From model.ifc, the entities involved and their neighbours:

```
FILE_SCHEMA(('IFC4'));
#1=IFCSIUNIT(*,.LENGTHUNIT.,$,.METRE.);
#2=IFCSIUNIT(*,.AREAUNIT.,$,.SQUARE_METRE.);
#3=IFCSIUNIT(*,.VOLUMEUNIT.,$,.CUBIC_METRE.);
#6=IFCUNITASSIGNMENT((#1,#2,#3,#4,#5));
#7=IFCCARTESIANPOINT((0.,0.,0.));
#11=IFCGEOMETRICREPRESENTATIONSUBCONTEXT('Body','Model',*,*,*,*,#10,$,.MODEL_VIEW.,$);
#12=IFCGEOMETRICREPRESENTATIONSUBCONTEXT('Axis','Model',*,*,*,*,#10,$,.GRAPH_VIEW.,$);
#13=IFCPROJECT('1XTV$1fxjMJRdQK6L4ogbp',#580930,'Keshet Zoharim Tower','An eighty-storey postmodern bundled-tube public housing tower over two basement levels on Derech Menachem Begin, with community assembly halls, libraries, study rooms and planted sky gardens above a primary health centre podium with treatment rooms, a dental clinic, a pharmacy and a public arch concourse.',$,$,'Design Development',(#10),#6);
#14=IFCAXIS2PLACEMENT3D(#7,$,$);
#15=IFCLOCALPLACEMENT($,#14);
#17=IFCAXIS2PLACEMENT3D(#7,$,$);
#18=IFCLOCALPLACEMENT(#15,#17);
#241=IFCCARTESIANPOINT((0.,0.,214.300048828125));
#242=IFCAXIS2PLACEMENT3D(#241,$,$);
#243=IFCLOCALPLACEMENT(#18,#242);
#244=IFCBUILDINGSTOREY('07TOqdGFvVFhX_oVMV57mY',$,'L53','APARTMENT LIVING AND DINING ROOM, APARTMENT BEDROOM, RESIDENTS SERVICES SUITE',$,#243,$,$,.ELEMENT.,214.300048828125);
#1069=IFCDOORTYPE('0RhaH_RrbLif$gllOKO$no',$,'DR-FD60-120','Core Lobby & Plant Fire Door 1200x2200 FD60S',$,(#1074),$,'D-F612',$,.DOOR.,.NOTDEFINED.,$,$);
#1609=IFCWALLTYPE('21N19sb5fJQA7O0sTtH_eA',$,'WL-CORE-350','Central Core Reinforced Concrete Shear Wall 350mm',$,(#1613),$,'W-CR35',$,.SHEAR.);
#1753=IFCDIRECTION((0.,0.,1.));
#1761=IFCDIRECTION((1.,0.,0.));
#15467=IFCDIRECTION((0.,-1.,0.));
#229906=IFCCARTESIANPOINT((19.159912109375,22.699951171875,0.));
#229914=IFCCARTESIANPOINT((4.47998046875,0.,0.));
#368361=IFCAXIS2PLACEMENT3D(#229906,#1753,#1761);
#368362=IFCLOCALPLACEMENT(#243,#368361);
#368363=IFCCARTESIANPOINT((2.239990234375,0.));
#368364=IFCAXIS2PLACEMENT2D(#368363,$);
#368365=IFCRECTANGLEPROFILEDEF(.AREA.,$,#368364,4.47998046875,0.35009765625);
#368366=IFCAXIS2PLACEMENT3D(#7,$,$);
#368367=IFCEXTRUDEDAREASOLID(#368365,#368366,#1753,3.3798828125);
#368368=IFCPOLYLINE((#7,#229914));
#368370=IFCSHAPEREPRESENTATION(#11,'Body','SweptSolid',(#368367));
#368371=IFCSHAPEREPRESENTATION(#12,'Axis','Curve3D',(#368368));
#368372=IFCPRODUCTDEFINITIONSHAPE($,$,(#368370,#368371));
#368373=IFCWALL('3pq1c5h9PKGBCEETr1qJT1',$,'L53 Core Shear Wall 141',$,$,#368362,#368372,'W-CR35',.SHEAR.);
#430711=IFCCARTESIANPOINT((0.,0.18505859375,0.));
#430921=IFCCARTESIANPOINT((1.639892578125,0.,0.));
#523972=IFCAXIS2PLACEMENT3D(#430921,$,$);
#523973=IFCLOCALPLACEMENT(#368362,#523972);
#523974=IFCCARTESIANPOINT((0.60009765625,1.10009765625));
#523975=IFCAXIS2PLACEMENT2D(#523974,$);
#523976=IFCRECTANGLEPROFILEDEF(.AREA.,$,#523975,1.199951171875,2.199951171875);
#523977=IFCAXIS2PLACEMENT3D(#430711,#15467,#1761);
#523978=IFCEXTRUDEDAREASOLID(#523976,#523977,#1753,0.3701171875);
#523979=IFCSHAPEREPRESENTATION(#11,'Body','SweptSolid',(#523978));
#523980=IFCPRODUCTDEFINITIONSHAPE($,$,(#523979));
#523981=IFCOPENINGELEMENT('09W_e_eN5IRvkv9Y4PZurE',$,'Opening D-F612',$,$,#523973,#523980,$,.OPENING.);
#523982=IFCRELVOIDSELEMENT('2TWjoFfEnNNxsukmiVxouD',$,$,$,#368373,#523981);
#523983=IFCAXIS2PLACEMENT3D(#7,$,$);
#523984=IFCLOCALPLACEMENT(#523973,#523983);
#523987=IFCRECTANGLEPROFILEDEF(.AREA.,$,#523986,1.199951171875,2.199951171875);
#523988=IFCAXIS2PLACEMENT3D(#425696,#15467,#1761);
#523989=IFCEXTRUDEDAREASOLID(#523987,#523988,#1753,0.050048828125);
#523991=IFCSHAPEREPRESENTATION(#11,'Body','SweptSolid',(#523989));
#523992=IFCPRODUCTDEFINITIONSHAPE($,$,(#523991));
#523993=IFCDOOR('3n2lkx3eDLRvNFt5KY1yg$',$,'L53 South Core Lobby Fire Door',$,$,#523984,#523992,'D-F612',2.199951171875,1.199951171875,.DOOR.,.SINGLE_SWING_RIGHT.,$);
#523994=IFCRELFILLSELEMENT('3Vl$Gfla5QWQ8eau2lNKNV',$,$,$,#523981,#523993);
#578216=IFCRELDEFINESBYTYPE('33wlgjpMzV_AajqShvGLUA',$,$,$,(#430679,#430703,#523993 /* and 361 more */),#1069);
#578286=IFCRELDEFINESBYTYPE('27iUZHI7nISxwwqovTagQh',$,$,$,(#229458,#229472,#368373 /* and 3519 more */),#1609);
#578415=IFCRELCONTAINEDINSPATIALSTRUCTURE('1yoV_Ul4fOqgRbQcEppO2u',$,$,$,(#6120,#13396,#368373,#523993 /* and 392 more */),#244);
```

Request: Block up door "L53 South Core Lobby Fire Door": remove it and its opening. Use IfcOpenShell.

```python
import ifcopenshell
import ifcopenshell.api.feature
import ifcopenshell.api.root
import ifcopenshell.geom
import ifcopenshell.util.shape

model = ifcopenshell.open("model.ifc")
settings = ifcopenshell.geom.settings()


def volume(element):
    """Net volume in cubic metres, openings subtracted."""
    shape = ifcopenshell.geom.create_shape(settings, element)
    return ifcopenshell.util.shape.get_volume(shape.geometry)


door = model.by_guid("3n2lkx3eDLRvNFt5KY1yg$")
opening = door.FillsVoids[0].RelatingOpeningElement
wall = opening.VoidsElements[0].RelatingBuildingElement
before = volume(wall)

ifcopenshell.api.root.remove_product(model, product=door)
ifcopenshell.api.feature.remove_feature(model, feature=opening)

after = volume(wall)

print(f"wall volume {before:.3f} -> {after:.3f} m3")

model.write("model-out.ifc")
```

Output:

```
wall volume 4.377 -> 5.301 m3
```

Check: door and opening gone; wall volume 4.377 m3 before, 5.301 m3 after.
